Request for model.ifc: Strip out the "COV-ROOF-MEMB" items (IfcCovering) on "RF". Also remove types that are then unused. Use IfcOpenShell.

First a look at what the model holds.

```python
import ifcopenshell
import ifcopenshell.util.element

model = ifcopenshell.open("model.ifc")
print(model.schema)
storey = next(s for s in model.by_type("IfcBuildingStorey") if s.Name == "RF")
coverings = [e for e in ifcopenshell.util.element.get_decomposition(storey) if e.is_a("IfcCovering")]
seen = {}
for e in coverings:
    element_type = ifcopenshell.util.element.get_type(e)
    name = element_type.Name if element_type not in (None, e) else None
    seen[name] = seen.get(name, 0) + 1
for name, count in sorted(seen.items(), key=str):
    print(count, "x", name)
```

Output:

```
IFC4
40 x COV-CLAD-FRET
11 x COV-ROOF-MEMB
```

```python
import ifcopenshell
import ifcopenshell.api.root
import ifcopenshell.util.element

model = ifcopenshell.open("model.ifc")

storey = next(s for s in model.by_type("IfcBuildingStorey") if s.Name == "RF")
coverings = [e for e in ifcopenshell.util.element.get_decomposition(storey) if e.is_a("IfcCovering")]
targets = [e for e in coverings if (t := ifcopenshell.util.element.get_type(e)) not in (None, e) and t.Name == "COV-ROOF-MEMB"]
types = {ifcopenshell.util.element.get_type(e) for e in targets} - {None, *targets}

for e in targets:
    ifcopenshell.api.root.remove_product(model, product=e)
print(len(targets), "removed")

unused = [t for t in types if not ifcopenshell.util.element.get_types(t)]
for t in unused:
    ifcopenshell.api.root.remove_product(model, product=t)
print(len(unused), "unused types removed")

model.write("model_updated.ifc")
```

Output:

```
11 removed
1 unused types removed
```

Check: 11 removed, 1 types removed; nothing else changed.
